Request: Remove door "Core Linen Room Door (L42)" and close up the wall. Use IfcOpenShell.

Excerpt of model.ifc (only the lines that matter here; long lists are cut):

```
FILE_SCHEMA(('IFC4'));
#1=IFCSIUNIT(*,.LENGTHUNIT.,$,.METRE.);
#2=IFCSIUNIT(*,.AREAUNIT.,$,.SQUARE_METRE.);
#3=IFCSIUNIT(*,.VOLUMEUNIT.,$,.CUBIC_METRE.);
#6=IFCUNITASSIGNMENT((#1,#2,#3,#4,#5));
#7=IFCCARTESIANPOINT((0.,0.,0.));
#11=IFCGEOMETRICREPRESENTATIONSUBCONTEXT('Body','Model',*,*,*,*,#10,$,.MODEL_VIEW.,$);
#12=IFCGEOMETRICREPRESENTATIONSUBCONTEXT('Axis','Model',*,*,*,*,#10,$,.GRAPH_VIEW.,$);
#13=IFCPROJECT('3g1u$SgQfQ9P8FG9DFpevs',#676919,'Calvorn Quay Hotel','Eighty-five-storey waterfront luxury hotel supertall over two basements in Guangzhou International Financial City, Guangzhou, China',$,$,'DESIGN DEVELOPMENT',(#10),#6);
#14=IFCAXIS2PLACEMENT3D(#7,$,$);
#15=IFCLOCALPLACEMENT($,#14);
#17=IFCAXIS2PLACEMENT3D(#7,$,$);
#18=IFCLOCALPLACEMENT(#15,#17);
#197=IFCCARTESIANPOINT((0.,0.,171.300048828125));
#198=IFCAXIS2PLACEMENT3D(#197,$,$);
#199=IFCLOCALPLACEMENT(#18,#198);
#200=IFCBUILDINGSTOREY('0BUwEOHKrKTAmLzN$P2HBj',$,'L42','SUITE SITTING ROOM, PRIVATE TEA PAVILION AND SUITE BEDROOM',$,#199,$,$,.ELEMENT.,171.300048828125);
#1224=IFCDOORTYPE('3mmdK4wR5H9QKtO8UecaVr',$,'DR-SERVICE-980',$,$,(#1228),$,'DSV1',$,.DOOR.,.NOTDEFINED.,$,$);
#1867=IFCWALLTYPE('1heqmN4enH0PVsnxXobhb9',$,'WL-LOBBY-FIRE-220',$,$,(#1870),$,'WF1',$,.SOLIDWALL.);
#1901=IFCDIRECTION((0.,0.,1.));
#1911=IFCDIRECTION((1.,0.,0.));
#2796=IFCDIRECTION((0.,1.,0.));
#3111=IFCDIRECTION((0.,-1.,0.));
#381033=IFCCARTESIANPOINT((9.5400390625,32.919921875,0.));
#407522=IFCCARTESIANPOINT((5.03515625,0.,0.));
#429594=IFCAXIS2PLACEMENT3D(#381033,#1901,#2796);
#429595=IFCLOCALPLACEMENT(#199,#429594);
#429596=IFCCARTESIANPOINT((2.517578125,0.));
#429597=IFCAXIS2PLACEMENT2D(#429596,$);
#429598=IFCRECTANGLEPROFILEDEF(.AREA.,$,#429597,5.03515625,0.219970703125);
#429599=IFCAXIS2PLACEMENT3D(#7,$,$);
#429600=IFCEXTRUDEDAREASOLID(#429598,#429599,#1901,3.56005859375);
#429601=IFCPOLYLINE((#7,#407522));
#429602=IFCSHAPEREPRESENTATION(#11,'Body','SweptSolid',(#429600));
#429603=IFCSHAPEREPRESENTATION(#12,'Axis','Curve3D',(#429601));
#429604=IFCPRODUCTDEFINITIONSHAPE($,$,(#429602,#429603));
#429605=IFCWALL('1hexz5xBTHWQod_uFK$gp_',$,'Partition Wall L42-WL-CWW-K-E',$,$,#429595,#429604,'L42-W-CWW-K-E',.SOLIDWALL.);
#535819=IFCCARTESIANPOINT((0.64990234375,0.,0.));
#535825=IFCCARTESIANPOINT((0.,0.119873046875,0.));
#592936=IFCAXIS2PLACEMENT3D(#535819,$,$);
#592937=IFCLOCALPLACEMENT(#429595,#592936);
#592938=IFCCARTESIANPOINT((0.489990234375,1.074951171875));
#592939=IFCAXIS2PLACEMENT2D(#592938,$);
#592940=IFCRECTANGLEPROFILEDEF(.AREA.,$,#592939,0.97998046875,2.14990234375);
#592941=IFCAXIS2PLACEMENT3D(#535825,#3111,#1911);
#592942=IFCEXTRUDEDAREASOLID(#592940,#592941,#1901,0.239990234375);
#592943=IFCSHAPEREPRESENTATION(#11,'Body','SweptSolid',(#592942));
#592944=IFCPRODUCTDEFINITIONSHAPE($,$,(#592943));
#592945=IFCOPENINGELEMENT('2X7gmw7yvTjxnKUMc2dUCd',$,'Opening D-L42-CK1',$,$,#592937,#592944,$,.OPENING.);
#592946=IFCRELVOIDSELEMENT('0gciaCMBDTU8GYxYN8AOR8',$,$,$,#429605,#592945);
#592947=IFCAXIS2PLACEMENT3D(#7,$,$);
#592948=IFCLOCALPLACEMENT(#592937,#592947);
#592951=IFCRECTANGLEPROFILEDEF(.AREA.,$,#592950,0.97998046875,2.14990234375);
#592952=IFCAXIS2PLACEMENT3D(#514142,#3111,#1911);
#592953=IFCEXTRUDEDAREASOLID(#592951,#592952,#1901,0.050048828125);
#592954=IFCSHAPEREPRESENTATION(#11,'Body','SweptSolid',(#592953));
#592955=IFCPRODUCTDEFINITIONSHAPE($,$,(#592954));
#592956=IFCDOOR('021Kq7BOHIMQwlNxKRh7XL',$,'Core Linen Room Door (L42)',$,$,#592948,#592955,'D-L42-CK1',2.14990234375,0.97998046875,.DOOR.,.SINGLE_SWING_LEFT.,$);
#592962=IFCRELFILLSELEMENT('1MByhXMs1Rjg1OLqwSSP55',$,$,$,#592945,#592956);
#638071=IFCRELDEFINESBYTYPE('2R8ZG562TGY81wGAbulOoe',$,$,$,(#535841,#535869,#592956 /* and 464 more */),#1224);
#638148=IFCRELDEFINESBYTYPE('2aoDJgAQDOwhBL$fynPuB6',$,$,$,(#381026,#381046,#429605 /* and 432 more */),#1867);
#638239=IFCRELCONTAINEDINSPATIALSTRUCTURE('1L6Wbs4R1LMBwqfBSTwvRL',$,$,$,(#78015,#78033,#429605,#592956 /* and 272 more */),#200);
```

```python
import ifcopenshell
import ifcopenshell.api.feature
import ifcopenshell.api.root
import ifcopenshell.geom
import ifcopenshell.util.shape

model = ifcopenshell.open("model.ifc")
settings = ifcopenshell.geom.settings()


def volume(element):
    """Net volume in cubic metres, openings subtracted."""
    shape = ifcopenshell.geom.create_shape(settings, element)
    return ifcopenshell.util.shape.get_volume(shape.geometry)


door = model.by_guid("021Kq7BOHIMQwlNxKRh7XL")
opening = door.FillsVoids[0].RelatingOpeningElement
wall = opening.VoidsElements[0].RelatingBuildingElement
before = volume(wall)

ifcopenshell.api.root.remove_product(model, product=door)
ifcopenshell.api.feature.remove_feature(model, feature=opening)

after = volume(wall)

print(f"wall volume {before:.3f} -> {after:.3f} m3")

model.write("model-out.ifc")
```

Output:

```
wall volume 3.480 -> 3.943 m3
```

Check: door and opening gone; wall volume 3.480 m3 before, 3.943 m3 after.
